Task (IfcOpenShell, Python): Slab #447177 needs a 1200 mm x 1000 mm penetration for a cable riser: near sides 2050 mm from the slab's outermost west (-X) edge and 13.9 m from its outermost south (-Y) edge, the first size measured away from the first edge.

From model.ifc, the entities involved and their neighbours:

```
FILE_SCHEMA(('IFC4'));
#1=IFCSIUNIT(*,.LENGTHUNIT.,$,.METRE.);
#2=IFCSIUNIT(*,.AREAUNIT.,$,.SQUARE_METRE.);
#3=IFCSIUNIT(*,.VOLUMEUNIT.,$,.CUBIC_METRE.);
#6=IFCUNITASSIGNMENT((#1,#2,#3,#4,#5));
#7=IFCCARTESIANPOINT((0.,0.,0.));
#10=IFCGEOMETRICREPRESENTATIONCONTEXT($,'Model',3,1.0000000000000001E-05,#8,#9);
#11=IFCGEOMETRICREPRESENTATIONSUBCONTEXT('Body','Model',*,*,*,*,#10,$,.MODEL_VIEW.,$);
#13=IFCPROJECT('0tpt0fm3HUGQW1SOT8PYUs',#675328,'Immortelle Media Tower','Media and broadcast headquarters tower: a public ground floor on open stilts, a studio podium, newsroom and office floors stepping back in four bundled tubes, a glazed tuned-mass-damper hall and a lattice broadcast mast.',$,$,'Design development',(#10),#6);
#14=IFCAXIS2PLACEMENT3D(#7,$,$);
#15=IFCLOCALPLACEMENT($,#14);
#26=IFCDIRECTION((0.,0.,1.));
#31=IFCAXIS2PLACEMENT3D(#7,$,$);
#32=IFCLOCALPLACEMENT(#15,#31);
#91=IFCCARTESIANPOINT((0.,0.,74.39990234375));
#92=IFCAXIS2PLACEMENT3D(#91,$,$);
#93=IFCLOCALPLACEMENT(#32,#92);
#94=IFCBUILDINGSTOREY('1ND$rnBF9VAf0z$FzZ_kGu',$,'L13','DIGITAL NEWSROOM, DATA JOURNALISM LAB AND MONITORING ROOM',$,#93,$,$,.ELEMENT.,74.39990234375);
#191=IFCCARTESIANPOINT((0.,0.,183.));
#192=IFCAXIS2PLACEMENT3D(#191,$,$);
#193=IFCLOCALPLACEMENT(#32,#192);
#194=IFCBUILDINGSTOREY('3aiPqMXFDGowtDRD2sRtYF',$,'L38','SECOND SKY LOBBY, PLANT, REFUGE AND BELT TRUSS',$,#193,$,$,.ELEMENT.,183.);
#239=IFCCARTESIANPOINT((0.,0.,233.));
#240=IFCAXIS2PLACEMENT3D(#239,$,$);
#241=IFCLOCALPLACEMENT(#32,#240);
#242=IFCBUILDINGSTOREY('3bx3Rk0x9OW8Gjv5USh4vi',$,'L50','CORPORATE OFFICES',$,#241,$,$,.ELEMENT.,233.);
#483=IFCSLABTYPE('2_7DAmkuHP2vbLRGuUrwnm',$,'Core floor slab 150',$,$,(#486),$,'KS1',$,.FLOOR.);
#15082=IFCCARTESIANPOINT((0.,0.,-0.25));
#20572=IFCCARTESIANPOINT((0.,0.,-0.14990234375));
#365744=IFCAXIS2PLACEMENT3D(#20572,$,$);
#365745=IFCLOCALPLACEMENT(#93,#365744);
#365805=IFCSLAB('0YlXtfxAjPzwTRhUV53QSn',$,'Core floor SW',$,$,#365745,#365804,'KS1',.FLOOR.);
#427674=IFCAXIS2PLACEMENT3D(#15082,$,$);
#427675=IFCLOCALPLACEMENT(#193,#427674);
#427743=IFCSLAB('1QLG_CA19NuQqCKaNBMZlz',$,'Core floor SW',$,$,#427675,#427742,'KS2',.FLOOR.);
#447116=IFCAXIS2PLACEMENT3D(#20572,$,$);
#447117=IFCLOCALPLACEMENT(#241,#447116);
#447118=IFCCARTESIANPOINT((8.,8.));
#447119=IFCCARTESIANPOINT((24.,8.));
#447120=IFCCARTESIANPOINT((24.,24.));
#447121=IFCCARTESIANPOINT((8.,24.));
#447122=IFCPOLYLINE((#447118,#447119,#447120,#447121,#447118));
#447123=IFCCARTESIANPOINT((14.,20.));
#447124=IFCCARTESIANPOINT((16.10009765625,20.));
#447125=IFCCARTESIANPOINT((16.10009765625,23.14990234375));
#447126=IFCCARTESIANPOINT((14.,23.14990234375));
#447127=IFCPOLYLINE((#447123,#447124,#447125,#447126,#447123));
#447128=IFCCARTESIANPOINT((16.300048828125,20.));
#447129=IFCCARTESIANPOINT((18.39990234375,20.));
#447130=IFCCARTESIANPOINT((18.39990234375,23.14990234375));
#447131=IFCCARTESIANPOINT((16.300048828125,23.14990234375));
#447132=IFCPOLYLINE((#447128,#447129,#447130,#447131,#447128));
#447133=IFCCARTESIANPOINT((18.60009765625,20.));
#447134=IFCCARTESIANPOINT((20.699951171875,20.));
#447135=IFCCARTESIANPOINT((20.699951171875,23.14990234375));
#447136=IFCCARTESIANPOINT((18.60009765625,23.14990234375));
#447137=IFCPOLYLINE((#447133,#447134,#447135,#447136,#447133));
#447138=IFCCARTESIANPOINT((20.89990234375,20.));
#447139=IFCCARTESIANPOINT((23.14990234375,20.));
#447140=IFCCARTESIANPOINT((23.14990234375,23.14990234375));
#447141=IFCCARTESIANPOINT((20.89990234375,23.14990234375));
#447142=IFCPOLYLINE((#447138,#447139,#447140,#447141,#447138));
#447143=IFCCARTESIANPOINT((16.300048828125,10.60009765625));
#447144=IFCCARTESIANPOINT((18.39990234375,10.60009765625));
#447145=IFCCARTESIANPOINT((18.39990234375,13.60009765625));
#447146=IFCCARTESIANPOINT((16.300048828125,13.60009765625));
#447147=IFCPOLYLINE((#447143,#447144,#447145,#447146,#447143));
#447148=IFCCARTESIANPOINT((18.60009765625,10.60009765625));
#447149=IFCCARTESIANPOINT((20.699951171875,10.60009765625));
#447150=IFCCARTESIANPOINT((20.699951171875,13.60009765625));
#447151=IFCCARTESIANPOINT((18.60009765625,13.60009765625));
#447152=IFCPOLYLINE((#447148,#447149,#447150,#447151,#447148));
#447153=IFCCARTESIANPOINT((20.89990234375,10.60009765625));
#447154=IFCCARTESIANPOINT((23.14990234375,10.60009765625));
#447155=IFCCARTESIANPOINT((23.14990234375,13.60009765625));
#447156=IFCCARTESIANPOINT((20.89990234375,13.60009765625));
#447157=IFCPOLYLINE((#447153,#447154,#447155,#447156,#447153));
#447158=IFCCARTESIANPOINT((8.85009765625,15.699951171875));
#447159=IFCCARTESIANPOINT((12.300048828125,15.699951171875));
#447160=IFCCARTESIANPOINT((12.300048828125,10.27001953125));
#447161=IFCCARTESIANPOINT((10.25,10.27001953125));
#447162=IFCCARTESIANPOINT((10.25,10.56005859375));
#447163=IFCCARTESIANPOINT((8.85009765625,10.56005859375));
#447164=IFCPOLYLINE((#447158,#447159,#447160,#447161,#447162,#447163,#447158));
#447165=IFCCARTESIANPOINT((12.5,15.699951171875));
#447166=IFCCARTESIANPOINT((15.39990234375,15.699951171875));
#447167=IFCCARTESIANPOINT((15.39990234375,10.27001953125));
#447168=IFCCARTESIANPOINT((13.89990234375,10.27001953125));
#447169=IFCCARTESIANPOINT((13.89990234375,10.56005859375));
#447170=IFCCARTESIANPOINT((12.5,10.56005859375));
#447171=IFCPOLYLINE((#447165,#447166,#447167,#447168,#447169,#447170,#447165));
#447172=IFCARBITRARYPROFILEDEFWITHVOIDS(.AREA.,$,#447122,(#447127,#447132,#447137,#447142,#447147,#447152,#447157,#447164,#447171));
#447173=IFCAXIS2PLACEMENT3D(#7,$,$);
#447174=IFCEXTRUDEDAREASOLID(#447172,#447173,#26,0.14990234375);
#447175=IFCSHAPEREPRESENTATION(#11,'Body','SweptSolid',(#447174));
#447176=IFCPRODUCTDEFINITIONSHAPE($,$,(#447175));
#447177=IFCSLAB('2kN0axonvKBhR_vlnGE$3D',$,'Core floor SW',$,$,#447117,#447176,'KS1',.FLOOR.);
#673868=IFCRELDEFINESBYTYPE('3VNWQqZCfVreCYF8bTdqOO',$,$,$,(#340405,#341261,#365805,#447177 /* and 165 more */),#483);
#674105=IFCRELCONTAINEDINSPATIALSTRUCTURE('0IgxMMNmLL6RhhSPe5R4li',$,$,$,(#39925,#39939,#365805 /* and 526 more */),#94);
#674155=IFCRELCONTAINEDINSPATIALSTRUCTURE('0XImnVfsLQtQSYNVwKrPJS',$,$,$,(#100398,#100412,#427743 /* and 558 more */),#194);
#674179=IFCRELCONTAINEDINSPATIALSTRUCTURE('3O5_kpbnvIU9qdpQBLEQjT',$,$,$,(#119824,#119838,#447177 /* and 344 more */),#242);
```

```python
import numpy as np
import ifcopenshell
import ifcopenshell.api.feature
import ifcopenshell.api.geometry
import ifcopenshell.api.root
import ifcopenshell.geom
import ifcopenshell.util.placement
import ifcopenshell.util.representation
import ifcopenshell.util.shape
import ifcopenshell.util.unit

model = ifcopenshell.open("model.ifc")
unit_scale = ifcopenshell.util.unit.calculate_unit_scale(model)
settings = ifcopenshell.geom.settings()


def volume(element):
    """Net volume in cubic metres, openings subtracted."""
    shape = ifcopenshell.geom.create_shape(settings, element)
    return ifcopenshell.util.shape.get_volume(shape.geometry)


slab = model.by_id(447177)
before = volume(slab)

# Extent in the slab's own axes, in metres. The edges named are its -X and -Y sides.
slab_shape = ifcopenshell.geom.create_shape(settings, slab)
vertices = ifcopenshell.util.shape.get_vertices(slab_shape.geometry)
x_min, y_min, bottom = vertices.min(axis=0)
top = vertices[:, 2].max()

opening = ifcopenshell.api.root.create_entity(model, ifc_class="IfcOpeningElement", name="Cable riser opening", predefined_type="OPENING")
context = ifcopenshell.util.representation.get_context(model, "Model", "Body", "MODEL_VIEW")
width, depth = 1.2, 1
outline = [(0.0, 0.0), (width, 0.0), (width, depth), (0.0, depth), (0.0, 0.0)]
# Overshoot both faces by 50 mm so the cut is clean.
shape = ifcopenshell.api.geometry.add_slab_representation(
    model, context=context, depth=top - bottom + 0.1, polyline=outline
)
ifcopenshell.api.geometry.assign_representation(model, product=opening, representation=shape)

matrix = ifcopenshell.util.placement.get_local_placement(slab.ObjectPlacement)
matrix[:, 3] = matrix @ np.append(np.array([x_min + 2.05, y_min + 13.9, bottom - 0.05]) / unit_scale, 1.0)
ifcopenshell.api.geometry.edit_object_placement(model, product=opening, matrix=matrix, is_si=False)
ifcopenshell.api.feature.add_feature(model, feature=opening, element=slab)

after = volume(slab)

print(f"slab volume {before:.3f} -> {after:.3f} m3")

model.write("model_v2.ifc")
```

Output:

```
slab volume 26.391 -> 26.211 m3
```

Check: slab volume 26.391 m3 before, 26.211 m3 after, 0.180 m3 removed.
